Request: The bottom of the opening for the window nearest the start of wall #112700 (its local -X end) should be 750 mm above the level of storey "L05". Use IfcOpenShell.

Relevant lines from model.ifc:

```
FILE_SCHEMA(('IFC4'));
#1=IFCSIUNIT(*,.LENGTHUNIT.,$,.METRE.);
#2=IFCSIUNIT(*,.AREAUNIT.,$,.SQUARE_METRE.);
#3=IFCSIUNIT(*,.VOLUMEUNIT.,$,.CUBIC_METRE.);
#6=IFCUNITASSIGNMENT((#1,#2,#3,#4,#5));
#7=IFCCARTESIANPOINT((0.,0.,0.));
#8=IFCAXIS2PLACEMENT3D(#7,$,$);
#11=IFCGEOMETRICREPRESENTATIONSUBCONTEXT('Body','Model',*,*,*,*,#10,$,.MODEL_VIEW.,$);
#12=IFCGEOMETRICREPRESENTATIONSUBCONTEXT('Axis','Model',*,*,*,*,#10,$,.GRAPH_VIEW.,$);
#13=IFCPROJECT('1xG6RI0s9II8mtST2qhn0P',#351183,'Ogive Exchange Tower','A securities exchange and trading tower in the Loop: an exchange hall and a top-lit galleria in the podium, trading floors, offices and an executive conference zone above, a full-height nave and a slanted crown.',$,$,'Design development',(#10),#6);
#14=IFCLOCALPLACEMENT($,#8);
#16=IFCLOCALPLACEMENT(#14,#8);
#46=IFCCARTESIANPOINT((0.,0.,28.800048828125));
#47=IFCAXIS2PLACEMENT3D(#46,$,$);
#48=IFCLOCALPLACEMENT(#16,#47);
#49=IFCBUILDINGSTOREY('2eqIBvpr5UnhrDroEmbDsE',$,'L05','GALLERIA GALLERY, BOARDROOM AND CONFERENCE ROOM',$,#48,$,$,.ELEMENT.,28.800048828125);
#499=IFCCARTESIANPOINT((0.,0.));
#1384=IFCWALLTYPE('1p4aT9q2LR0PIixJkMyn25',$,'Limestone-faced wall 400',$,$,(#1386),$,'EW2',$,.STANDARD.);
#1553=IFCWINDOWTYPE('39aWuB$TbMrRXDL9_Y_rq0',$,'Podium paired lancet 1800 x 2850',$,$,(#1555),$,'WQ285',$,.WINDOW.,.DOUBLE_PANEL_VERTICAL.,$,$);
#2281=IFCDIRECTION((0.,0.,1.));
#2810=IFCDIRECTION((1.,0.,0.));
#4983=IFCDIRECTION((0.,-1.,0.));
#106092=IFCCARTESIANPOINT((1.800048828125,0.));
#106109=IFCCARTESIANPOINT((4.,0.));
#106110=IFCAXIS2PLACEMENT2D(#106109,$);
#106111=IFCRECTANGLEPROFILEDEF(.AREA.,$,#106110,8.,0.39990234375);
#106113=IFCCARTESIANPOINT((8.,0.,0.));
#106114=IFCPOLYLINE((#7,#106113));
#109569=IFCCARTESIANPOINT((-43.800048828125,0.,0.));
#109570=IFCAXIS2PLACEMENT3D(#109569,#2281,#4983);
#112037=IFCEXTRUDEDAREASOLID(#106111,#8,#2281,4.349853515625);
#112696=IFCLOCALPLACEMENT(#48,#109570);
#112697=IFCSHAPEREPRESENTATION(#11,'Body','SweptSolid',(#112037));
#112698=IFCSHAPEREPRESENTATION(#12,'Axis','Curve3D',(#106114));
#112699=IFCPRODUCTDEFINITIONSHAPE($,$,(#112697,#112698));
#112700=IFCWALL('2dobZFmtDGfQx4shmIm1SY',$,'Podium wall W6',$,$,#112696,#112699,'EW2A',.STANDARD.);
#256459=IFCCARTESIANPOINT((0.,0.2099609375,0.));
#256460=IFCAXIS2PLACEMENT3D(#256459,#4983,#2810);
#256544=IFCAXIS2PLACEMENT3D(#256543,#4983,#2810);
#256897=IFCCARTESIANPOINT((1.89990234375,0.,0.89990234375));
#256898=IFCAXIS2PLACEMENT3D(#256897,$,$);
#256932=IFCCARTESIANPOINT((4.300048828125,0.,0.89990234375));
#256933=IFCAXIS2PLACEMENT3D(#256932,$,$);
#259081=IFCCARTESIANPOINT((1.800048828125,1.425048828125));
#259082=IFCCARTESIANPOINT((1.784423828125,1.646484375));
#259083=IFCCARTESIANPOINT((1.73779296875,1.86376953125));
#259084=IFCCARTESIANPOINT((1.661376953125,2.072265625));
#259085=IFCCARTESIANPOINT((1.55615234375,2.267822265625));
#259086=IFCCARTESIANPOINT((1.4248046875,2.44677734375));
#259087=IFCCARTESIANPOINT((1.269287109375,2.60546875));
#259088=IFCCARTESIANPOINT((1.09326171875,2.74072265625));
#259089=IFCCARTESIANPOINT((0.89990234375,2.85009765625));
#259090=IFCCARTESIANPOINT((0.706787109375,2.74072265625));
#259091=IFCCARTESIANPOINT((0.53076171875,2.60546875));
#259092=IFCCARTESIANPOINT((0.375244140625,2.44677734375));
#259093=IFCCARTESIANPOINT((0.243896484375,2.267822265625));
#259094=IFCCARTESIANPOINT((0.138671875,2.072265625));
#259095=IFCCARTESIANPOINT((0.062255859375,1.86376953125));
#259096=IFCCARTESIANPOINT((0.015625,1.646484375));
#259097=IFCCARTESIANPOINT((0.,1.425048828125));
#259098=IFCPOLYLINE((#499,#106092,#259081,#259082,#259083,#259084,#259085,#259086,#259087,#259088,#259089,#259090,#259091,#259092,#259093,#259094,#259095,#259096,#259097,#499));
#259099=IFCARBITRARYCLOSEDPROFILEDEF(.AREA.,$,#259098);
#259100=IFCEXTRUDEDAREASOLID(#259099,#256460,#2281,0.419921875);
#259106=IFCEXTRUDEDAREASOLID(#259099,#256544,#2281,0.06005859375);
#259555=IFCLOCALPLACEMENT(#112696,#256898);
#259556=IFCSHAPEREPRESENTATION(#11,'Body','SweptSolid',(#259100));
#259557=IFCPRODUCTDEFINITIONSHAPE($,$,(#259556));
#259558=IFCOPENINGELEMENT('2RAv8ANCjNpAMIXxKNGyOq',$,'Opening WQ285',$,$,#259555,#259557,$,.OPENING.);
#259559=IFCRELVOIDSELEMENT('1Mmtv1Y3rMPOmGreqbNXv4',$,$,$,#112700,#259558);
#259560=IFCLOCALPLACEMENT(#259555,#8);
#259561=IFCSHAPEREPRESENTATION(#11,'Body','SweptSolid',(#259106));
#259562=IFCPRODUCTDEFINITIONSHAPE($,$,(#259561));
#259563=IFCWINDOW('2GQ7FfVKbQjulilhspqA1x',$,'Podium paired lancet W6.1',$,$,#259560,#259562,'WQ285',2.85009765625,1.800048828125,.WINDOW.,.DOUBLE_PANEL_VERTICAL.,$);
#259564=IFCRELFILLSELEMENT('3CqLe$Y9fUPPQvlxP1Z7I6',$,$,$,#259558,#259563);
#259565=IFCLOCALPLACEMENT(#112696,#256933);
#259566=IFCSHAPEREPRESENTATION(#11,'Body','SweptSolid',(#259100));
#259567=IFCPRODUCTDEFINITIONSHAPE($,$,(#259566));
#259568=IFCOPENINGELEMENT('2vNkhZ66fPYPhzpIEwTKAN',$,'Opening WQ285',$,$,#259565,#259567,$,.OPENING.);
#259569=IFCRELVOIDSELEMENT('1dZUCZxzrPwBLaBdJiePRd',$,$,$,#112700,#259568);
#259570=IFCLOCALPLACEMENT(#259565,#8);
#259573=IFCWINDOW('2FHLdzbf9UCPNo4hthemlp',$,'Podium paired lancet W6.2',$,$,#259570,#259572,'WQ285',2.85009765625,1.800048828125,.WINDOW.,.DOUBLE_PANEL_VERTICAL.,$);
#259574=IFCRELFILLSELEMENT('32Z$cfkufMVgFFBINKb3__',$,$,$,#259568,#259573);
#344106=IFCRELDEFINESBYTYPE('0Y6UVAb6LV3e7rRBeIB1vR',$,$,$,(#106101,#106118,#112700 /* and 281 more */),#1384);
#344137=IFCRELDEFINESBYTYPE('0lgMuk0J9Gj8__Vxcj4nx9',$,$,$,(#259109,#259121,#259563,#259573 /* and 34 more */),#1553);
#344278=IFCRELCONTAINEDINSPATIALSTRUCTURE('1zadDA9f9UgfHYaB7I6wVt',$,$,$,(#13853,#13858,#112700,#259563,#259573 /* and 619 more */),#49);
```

```python
import numpy as np
import ifcopenshell
import ifcopenshell.api.geometry
import ifcopenshell.geom
import ifcopenshell.util.element
import ifcopenshell.util.placement
import ifcopenshell.util.shape
import ifcopenshell.util.unit

model = ifcopenshell.open("model.ifc")
unit_scale = ifcopenshell.util.unit.calculate_unit_scale(model)

window = model.by_guid("2GQ7FfVKbQjulilhspqA1x")
opening = window.FillsVoids[0].RelatingOpeningElement
storey = ifcopenshell.util.element.get_container(window, ifc_class="IfcBuildingStorey")
level = ifcopenshell.util.placement.get_local_placement(storey.ObjectPlacement)[2, 3]

# The opening's origin need not be at the sill, so measure its lowest point.
shape = ifcopenshell.geom.create_shape(ifcopenshell.geom.settings(), opening)
bottom = ifcopenshell.util.shape.get_shape_bottom_elevation(shape, shape.geometry) / unit_scale
dz = level + 0.75 - bottom

shift = np.array([0.0, 0.0, dz])
# The window is placed relative to its opening, so it follows when the opening moves.
matrix = ifcopenshell.util.placement.get_local_placement(opening.ObjectPlacement)
matrix[:3, 3] += shift
ifcopenshell.api.geometry.edit_object_placement(
    model, product=opening, matrix=matrix, is_si=False, should_transform_children=True
)

print(f"moved by {dz * unit_scale:+.3f} m")

model.write("model_v2.ifc")
```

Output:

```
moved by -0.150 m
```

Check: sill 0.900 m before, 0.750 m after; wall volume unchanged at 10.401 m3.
